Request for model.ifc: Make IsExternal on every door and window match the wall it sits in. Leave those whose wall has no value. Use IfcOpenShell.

First a look at what the model holds.

```python
import ifcopenshell
import ifcopenshell.util.element

model = ifcopenshell.open("model.ifc")
print(model.schema)
seen = {}
for e in model.by_type("IfcDoor") + model.by_type("IfcWindow"):
    if not e.FillsVoids:
        continue
    host = e.FillsVoids[0].RelatingOpeningElement.VoidsElements[0].RelatingBuildingElement
    own = ifcopenshell.util.element.get_pset(e, f"Pset_{e.is_a()[3:].removesuffix('StandardCase')}Common", "IsExternal")
    wall = ifcopenshell.util.element.get_pset(host, "Pset_WallCommon", "IsExternal")
    seen[e.is_a(), own, wall] = seen.get((e.is_a(), own, wall), 0) + 1
for (cls, own, wall), count in sorted(seen.items(), key=str):
    print(count, cls, "IsExternal:", own, "| host wall:", wall)
```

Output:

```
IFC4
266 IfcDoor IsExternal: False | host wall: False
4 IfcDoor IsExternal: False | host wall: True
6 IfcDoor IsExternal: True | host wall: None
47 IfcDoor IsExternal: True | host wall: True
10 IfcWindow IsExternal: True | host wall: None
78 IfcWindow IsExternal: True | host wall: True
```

```python
import ifcopenshell
import ifcopenshell.api.pset
import ifcopenshell.util.element

model = ifcopenshell.open("model.ifc")

count = 0
for ifc_class, pset_name in (("IfcDoor", "Pset_DoorCommon"), ("IfcWindow", "Pset_WindowCommon")):
    for e in model.by_type(ifc_class):
        if not e.FillsVoids:
            continue
        host = e.FillsVoids[0].RelatingOpeningElement.VoidsElements[0].RelatingBuildingElement
        external = ifcopenshell.util.element.get_pset(host, "Pset_WallCommon", "IsExternal")
        if external is None or ifcopenshell.util.element.get_pset(e, pset_name, "IsExternal") == external:
            continue
        pset = ifcopenshell.api.pset.add_pset(model, product=e, name=pset_name)
        ifcopenshell.api.pset.edit_pset(model, pset=pset, properties={"IsExternal": external})
        count += 1

print(count, "updated")

model.write("model_updated.ifc")
```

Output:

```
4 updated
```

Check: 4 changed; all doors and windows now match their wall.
